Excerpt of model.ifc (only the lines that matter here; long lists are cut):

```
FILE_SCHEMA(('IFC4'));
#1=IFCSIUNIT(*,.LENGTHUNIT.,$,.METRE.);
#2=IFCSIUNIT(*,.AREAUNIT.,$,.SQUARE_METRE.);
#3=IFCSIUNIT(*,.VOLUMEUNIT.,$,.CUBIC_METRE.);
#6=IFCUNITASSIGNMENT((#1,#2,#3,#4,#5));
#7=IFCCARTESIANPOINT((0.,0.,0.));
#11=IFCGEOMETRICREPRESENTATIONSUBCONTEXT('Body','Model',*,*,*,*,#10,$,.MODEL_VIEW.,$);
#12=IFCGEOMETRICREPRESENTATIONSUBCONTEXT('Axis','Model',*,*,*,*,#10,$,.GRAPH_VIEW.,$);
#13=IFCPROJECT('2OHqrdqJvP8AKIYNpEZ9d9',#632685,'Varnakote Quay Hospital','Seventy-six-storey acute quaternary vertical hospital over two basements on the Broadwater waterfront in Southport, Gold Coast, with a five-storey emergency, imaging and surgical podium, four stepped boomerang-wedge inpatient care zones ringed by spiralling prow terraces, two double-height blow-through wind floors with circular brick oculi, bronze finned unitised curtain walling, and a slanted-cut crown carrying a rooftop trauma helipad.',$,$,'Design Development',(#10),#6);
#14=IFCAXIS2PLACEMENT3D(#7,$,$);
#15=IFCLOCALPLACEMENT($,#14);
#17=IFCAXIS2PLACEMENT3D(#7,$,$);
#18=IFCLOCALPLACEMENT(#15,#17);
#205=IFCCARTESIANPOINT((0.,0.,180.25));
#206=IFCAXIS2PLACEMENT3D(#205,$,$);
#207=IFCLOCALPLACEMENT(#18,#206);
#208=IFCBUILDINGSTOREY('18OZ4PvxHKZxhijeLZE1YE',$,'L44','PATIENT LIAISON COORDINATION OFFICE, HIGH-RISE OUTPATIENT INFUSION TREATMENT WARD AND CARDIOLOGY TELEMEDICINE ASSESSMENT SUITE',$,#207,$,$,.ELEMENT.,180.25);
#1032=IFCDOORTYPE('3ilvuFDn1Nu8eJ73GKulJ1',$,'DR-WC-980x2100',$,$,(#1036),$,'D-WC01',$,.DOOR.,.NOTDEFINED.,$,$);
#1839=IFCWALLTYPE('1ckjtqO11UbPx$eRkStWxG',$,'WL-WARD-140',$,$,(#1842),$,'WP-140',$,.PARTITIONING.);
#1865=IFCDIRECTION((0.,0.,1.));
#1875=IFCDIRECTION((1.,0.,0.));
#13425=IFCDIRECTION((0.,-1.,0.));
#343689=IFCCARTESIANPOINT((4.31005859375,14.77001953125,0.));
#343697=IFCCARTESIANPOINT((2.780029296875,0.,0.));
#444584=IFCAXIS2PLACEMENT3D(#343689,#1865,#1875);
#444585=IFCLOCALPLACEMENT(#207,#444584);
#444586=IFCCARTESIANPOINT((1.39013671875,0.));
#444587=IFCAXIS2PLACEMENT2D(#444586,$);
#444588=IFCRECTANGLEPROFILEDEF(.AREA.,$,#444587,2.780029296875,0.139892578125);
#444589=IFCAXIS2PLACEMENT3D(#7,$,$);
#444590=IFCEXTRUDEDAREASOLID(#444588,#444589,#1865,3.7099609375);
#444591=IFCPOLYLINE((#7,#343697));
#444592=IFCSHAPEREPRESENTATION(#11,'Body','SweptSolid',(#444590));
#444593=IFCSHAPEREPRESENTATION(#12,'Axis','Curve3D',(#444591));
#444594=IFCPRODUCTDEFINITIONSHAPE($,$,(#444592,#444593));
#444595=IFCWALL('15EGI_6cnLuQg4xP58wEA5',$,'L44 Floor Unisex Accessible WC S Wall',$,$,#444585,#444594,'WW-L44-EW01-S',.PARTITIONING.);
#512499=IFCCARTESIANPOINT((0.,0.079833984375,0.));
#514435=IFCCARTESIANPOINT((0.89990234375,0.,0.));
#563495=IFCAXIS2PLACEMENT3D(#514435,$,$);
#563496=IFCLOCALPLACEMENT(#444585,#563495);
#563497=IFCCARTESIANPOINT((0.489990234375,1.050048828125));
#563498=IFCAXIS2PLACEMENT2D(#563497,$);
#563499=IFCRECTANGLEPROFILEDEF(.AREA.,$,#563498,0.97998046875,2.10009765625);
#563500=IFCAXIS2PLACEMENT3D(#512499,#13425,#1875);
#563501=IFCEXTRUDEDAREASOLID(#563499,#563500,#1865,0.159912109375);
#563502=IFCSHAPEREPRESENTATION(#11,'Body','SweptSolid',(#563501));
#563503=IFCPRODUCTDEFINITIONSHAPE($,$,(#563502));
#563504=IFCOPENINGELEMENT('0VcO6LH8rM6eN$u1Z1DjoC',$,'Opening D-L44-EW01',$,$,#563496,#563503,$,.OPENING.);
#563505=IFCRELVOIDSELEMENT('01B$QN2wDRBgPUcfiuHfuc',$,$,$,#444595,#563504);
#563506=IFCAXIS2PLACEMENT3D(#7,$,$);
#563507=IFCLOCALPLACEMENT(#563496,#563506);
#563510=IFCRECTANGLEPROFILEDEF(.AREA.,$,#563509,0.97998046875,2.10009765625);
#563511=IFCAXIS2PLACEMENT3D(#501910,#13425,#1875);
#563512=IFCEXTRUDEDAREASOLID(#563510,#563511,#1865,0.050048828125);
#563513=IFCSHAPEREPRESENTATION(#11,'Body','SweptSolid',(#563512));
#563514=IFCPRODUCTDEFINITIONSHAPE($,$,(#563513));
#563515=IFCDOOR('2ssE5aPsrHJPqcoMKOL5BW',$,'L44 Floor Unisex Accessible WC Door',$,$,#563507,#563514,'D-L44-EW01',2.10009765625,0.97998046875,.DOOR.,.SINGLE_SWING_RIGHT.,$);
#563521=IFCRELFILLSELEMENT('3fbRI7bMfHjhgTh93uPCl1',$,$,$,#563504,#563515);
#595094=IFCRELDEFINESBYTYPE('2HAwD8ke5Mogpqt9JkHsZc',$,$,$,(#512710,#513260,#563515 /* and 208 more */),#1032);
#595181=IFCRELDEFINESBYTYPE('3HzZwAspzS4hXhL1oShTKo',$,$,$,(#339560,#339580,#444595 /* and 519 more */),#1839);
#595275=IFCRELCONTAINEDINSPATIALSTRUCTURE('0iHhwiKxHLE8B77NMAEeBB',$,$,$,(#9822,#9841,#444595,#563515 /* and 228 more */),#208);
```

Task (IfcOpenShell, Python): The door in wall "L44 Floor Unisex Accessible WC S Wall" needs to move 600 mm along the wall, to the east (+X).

```python
import ifcopenshell
import ifcopenshell.api.geometry
import ifcopenshell.util.placement
import ifcopenshell.util.unit

model = ifcopenshell.open("model.ifc")
unit_scale = ifcopenshell.util.unit.calculate_unit_scale(model)

door = model.by_guid("2ssE5aPsrHJPqcoMKOL5BW")
opening = door.FillsVoids[0].RelatingOpeningElement
wall = opening.VoidsElements[0].RelatingBuildingElement

wall_matrix = ifcopenshell.util.placement.get_local_placement(wall.ObjectPlacement)
shift = wall_matrix[:3, 0] * 0.6 / unit_scale
before = ifcopenshell.util.placement.get_local_placement(door.ObjectPlacement)[:3, 3].copy()

# The door is placed relative to its opening, so it follows when the opening moves.
matrix = ifcopenshell.util.placement.get_local_placement(opening.ObjectPlacement)
matrix[:3, 3] += shift
ifcopenshell.api.geometry.edit_object_placement(
    model, product=opening, matrix=matrix, is_si=False, should_transform_children=True
)

after = ifcopenshell.util.placement.get_local_placement(door.ObjectPlacement)[:3, 3]
print("door moved by", (after - before).round(3) + 0.0)

model.write("model_updated.ifc")
```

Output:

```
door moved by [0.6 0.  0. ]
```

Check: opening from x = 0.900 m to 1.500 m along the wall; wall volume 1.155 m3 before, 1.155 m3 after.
